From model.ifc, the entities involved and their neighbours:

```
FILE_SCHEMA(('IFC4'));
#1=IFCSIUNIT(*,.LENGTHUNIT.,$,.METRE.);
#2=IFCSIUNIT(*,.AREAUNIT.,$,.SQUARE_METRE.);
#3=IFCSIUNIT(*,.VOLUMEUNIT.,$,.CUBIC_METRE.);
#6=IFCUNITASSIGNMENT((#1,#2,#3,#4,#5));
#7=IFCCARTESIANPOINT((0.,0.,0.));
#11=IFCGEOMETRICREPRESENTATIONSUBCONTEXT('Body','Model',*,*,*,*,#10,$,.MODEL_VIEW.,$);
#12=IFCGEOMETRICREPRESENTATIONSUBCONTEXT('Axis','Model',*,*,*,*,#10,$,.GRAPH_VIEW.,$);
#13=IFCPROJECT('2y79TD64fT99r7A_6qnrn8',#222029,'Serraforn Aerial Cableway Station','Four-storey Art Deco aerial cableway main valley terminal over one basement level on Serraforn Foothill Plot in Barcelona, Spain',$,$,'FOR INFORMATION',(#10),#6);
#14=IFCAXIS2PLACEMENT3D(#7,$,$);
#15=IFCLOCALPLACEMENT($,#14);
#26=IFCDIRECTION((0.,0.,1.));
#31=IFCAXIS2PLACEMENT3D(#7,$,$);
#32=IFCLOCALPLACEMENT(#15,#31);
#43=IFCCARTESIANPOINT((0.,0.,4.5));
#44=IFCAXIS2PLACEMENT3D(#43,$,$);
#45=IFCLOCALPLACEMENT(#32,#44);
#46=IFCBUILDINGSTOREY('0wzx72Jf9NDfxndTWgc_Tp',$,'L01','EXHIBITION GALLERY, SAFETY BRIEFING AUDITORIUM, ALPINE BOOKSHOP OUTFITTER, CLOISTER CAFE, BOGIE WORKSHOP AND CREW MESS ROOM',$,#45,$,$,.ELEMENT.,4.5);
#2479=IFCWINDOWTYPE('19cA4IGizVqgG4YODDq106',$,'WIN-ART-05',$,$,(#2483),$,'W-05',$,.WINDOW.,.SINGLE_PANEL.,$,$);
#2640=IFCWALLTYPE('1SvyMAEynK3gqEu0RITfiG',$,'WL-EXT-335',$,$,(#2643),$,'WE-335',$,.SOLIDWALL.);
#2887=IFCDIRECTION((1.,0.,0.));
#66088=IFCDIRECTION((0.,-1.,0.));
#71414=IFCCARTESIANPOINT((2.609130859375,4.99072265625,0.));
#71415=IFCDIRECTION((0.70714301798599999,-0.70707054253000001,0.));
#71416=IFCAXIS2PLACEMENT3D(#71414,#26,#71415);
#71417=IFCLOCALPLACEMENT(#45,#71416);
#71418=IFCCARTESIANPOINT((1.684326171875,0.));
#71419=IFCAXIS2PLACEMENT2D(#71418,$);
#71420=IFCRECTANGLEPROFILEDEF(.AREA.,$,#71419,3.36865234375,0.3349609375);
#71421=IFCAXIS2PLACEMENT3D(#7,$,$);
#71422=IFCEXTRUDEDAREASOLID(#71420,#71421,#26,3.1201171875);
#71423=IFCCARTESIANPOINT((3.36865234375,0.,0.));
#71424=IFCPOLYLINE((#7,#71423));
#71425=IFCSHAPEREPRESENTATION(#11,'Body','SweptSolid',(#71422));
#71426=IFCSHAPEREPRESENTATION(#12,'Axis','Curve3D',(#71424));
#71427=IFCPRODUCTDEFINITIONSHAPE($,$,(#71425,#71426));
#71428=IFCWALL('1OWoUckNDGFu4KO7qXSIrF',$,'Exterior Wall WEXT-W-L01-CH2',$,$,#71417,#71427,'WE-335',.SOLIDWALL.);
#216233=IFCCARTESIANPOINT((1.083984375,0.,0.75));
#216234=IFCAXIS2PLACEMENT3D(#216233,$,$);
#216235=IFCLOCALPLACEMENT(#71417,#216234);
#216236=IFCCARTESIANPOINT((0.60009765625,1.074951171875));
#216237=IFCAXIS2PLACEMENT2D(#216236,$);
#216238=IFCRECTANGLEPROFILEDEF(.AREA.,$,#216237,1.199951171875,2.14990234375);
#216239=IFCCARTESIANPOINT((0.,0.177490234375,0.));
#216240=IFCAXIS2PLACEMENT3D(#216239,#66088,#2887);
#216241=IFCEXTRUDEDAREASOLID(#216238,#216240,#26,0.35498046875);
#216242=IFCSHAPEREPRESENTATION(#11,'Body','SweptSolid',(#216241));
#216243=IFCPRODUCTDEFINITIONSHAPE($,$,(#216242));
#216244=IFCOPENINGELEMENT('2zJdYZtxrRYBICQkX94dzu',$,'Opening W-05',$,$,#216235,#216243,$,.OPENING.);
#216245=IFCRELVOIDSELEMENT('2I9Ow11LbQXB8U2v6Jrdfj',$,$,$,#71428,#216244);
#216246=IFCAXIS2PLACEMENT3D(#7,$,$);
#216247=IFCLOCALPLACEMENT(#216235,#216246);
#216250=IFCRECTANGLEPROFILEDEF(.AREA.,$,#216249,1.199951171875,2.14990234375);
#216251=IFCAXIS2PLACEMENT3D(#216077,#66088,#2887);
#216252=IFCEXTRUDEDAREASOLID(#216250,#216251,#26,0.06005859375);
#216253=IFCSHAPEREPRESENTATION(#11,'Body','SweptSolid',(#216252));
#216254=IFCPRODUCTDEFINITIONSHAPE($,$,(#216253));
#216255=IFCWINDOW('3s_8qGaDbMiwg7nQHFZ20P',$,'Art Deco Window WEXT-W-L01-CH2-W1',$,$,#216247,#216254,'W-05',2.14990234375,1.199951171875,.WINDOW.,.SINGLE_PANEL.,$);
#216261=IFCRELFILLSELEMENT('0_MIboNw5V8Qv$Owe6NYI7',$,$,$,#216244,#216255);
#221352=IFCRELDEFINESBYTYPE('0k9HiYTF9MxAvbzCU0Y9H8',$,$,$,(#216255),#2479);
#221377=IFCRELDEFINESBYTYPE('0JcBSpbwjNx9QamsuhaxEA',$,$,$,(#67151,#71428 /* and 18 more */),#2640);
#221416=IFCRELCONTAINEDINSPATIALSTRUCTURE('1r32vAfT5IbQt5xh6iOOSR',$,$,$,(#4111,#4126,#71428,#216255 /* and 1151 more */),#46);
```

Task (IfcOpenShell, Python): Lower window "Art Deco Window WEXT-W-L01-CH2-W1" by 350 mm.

```python
import numpy as np
import ifcopenshell
import ifcopenshell.api.geometry
import ifcopenshell.util.placement
import ifcopenshell.util.unit

model = ifcopenshell.open("model.ifc")
unit_scale = ifcopenshell.util.unit.calculate_unit_scale(model)

window = model.by_guid("3s_8qGaDbMiwg7nQHFZ20P")
opening = window.FillsVoids[0].RelatingOpeningElement
dz = -0.35

shift = np.array([0.0, 0.0, dz])
# The window is placed relative to its opening, so it follows when the opening moves.
matrix = ifcopenshell.util.placement.get_local_placement(opening.ObjectPlacement)
matrix[:3, 3] += shift
ifcopenshell.api.geometry.edit_object_placement(
    model, product=opening, matrix=matrix, is_si=False, should_transform_children=True
)

print(f"moved by {dz * unit_scale:+.3f} m")

model.write("model_v2.ifc")
```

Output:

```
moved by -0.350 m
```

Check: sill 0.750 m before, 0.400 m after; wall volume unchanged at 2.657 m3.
